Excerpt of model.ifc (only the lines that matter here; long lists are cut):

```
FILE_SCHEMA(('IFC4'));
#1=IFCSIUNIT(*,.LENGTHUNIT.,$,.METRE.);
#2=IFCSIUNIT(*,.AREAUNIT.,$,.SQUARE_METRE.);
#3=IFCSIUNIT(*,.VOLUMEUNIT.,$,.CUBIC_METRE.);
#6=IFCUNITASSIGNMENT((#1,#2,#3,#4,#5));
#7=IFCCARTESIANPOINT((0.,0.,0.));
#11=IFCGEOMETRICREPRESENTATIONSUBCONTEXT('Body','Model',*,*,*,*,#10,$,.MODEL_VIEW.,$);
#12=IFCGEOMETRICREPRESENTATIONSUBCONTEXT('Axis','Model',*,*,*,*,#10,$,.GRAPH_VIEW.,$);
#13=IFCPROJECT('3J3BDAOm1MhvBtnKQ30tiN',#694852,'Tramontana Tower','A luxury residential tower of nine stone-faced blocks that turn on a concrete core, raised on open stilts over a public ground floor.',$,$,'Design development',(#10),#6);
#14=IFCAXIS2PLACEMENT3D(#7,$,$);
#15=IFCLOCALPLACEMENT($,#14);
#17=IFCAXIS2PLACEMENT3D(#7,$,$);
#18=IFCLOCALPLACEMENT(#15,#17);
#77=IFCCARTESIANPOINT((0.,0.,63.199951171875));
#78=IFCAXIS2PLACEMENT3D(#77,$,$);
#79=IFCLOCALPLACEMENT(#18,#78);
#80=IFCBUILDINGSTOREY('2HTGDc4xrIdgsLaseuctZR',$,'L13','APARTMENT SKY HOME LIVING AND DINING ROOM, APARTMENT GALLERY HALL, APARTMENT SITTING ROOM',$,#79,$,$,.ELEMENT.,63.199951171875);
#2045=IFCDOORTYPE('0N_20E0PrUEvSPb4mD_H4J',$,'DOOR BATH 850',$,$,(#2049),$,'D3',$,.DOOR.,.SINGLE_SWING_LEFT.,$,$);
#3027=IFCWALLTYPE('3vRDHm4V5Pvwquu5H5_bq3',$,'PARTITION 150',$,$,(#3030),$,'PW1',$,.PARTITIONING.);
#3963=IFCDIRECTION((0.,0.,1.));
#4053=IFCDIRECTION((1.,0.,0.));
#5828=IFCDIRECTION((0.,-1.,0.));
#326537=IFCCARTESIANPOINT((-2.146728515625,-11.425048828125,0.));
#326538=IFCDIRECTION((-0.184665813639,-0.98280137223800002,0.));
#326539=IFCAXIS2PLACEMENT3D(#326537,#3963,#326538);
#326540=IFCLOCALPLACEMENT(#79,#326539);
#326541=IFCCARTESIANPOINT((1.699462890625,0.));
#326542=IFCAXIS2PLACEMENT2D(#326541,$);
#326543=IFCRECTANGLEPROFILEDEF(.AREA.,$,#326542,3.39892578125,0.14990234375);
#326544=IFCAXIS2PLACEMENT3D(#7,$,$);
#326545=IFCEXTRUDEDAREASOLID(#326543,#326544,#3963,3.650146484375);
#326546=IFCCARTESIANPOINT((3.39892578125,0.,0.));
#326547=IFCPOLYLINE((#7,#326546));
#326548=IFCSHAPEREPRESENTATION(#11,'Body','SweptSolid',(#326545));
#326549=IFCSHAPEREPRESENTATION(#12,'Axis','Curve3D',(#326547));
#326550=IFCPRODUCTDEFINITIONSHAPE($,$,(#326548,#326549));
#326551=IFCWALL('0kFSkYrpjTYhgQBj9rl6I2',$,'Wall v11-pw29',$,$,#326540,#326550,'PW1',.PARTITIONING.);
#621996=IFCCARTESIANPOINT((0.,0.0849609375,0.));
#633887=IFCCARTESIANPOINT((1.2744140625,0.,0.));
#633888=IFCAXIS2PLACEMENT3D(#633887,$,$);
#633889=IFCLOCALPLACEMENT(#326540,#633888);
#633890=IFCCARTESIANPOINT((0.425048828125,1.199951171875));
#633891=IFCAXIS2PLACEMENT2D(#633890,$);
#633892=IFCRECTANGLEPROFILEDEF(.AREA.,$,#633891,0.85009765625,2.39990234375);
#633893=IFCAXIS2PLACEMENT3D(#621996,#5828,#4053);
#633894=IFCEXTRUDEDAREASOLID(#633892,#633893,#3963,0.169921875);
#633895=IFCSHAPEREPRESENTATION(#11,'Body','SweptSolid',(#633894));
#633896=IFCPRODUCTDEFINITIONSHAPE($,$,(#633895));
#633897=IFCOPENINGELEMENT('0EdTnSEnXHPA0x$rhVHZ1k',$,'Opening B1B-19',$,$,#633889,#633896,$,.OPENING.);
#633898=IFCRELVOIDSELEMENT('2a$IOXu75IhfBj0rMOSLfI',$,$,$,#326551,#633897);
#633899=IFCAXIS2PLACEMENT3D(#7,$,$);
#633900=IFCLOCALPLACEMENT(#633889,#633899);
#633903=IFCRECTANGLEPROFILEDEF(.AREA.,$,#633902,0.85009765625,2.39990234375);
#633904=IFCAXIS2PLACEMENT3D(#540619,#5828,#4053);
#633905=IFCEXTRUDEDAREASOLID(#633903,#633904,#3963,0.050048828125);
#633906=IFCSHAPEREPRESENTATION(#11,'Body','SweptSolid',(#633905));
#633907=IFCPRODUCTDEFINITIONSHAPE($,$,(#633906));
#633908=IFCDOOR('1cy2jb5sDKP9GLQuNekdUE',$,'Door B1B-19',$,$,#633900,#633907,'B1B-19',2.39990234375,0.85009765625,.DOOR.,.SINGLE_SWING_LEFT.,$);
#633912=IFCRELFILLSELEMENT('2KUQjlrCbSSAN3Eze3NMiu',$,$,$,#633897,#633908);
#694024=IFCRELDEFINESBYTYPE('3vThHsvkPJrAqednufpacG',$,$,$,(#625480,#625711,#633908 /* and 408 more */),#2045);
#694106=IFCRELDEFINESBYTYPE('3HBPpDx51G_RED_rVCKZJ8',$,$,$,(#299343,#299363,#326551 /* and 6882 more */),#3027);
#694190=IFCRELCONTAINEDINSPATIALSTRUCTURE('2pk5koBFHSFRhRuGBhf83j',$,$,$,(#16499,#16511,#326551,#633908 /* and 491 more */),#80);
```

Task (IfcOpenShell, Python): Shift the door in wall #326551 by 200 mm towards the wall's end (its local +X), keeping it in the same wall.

```python
import ifcopenshell
import ifcopenshell.api.geometry
import ifcopenshell.util.placement
import ifcopenshell.util.unit

model = ifcopenshell.open("model.ifc")
unit_scale = ifcopenshell.util.unit.calculate_unit_scale(model)

door = model.by_id(633908)
opening = door.FillsVoids[0].RelatingOpeningElement
wall = opening.VoidsElements[0].RelatingBuildingElement

wall_matrix = ifcopenshell.util.placement.get_local_placement(wall.ObjectPlacement)
shift = wall_matrix[:3, 0] * 0.2 / unit_scale
before = ifcopenshell.util.placement.get_local_placement(door.ObjectPlacement)[:3, 3].copy()

# The door is placed relative to its opening, so it follows when the opening moves.
matrix = ifcopenshell.util.placement.get_local_placement(opening.ObjectPlacement)
matrix[:3, 3] += shift
ifcopenshell.api.geometry.edit_object_placement(
    model, product=opening, matrix=matrix, is_si=False, should_transform_children=True
)

after = ifcopenshell.util.placement.get_local_placement(door.ObjectPlacement)[:3, 3]
print("door moved by", (after - before).round(3) + 0.0)

model.write("model_updated.ifc")
```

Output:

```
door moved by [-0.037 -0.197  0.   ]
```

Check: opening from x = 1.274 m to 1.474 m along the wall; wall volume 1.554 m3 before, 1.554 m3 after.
